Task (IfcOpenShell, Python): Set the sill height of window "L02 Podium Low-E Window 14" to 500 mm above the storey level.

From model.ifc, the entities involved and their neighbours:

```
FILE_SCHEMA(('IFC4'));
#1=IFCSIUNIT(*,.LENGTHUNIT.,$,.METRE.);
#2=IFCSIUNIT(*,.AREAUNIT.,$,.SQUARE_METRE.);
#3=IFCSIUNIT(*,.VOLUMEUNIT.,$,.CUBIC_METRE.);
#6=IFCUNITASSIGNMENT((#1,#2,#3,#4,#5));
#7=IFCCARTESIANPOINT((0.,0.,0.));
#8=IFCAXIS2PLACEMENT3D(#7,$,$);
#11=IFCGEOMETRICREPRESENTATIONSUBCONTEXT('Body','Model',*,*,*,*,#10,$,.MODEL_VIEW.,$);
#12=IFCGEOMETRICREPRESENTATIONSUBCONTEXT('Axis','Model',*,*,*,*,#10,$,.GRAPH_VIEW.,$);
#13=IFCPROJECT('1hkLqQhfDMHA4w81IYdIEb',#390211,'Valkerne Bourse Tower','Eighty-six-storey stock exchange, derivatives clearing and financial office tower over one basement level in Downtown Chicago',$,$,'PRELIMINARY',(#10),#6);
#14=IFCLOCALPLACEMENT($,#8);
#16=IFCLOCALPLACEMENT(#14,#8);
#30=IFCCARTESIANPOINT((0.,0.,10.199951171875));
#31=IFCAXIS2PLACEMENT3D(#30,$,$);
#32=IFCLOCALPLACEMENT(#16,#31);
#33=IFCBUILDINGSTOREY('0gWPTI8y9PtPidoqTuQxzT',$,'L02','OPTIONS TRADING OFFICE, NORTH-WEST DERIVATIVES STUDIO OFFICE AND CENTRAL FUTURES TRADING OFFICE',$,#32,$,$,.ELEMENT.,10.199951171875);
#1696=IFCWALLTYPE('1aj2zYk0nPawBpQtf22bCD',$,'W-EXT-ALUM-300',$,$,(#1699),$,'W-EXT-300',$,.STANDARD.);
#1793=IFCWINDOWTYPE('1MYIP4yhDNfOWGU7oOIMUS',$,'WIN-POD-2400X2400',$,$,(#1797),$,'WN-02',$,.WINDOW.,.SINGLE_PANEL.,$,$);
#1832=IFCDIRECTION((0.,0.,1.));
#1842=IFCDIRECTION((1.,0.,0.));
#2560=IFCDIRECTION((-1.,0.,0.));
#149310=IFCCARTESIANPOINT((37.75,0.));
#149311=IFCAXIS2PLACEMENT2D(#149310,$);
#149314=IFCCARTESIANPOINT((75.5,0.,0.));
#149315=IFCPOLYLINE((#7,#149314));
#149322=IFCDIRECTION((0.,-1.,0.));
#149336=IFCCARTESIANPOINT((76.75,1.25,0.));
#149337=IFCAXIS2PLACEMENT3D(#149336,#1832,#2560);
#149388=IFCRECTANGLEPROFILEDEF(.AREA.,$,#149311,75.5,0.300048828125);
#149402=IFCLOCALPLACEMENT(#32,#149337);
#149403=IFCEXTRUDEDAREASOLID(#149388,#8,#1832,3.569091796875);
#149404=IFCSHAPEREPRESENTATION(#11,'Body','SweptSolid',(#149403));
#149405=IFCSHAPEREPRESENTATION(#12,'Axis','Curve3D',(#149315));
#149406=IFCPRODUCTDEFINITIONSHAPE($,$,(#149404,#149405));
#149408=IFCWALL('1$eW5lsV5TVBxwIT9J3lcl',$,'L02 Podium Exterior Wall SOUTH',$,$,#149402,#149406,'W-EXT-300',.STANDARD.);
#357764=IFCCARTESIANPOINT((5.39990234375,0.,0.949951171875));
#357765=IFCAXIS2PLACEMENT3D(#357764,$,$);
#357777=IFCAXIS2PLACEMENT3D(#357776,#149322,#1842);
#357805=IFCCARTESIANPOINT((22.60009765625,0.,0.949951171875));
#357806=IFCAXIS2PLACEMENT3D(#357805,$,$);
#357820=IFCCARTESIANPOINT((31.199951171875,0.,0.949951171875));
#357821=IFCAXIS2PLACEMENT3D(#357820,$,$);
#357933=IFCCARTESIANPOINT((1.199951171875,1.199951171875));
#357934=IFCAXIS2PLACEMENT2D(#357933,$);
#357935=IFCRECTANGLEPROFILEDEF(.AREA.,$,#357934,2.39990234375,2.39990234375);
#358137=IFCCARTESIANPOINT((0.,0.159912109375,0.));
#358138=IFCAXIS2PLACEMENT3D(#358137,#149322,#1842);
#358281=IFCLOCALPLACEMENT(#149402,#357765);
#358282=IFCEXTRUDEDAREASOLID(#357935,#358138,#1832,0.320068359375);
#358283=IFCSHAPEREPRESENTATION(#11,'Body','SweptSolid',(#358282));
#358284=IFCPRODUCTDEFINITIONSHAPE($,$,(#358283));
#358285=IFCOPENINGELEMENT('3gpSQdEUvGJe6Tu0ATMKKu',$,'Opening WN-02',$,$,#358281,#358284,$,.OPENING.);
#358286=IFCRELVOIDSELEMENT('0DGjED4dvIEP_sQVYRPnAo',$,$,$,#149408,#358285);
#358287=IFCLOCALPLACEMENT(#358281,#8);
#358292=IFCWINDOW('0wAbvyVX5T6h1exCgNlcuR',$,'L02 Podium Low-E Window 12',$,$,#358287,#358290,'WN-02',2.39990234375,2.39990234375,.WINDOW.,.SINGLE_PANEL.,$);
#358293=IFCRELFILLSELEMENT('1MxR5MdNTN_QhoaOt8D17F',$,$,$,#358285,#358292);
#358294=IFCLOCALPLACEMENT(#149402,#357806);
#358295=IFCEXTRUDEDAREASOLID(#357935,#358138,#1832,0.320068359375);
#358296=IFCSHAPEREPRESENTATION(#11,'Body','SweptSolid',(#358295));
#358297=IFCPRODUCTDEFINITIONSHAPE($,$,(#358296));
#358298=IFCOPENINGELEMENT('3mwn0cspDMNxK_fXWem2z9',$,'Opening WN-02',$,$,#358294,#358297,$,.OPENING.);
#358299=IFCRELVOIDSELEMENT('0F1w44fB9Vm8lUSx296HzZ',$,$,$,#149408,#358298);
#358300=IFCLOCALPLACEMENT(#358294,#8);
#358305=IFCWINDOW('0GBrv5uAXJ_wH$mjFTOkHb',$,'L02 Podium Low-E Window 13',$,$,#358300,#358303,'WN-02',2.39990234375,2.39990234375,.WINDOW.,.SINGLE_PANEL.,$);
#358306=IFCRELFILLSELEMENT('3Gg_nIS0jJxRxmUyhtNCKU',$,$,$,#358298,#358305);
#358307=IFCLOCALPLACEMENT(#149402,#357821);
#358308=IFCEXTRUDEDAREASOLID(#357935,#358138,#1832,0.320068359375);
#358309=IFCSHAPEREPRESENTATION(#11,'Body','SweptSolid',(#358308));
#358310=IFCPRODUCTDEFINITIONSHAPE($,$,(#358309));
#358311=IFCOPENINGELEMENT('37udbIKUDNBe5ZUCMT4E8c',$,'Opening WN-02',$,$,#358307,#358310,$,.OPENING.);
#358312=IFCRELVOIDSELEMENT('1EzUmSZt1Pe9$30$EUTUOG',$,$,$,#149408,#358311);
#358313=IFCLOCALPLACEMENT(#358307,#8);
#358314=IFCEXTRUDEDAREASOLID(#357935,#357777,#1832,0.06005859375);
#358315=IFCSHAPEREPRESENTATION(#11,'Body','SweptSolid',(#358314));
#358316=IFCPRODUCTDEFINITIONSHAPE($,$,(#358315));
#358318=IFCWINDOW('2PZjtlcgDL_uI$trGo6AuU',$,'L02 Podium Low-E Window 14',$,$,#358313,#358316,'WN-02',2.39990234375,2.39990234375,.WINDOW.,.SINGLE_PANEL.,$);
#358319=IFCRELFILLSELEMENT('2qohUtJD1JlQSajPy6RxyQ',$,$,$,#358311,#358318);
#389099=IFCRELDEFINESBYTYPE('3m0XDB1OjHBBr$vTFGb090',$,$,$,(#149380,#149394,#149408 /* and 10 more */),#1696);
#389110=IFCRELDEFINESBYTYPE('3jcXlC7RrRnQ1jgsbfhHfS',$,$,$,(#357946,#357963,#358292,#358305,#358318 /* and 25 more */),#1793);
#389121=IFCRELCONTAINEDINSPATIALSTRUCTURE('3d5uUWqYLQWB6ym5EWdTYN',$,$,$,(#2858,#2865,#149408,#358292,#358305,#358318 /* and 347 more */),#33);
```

```python
import numpy as np
import ifcopenshell
import ifcopenshell.api.geometry
import ifcopenshell.geom
import ifcopenshell.util.element
import ifcopenshell.util.placement
import ifcopenshell.util.shape
import ifcopenshell.util.unit

model = ifcopenshell.open("model.ifc")
unit_scale = ifcopenshell.util.unit.calculate_unit_scale(model)

window = model.by_id(358318)
opening = window.FillsVoids[0].RelatingOpeningElement
storey = ifcopenshell.util.element.get_container(window, ifc_class="IfcBuildingStorey")
level = ifcopenshell.util.placement.get_local_placement(storey.ObjectPlacement)[2, 3]

# The opening's origin need not be at the sill, so measure its lowest point.
shape = ifcopenshell.geom.create_shape(ifcopenshell.geom.settings(), opening)
bottom = ifcopenshell.util.shape.get_shape_bottom_elevation(shape, shape.geometry) / unit_scale
dz = level + 0.5 / unit_scale - bottom

shift = np.array([0.0, 0.0, dz])
# The window is placed relative to its opening, so it follows when the opening moves.
matrix = ifcopenshell.util.placement.get_local_placement(opening.ObjectPlacement)
matrix[:3, 3] += shift
ifcopenshell.api.geometry.edit_object_placement(
    model, product=opening, matrix=matrix, is_si=False, should_transform_children=True
)

print(f"moved by {dz * unit_scale:+.3f} m")

model.write("model_updated.ifc")
```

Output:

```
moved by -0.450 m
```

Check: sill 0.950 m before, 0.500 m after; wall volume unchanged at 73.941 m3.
